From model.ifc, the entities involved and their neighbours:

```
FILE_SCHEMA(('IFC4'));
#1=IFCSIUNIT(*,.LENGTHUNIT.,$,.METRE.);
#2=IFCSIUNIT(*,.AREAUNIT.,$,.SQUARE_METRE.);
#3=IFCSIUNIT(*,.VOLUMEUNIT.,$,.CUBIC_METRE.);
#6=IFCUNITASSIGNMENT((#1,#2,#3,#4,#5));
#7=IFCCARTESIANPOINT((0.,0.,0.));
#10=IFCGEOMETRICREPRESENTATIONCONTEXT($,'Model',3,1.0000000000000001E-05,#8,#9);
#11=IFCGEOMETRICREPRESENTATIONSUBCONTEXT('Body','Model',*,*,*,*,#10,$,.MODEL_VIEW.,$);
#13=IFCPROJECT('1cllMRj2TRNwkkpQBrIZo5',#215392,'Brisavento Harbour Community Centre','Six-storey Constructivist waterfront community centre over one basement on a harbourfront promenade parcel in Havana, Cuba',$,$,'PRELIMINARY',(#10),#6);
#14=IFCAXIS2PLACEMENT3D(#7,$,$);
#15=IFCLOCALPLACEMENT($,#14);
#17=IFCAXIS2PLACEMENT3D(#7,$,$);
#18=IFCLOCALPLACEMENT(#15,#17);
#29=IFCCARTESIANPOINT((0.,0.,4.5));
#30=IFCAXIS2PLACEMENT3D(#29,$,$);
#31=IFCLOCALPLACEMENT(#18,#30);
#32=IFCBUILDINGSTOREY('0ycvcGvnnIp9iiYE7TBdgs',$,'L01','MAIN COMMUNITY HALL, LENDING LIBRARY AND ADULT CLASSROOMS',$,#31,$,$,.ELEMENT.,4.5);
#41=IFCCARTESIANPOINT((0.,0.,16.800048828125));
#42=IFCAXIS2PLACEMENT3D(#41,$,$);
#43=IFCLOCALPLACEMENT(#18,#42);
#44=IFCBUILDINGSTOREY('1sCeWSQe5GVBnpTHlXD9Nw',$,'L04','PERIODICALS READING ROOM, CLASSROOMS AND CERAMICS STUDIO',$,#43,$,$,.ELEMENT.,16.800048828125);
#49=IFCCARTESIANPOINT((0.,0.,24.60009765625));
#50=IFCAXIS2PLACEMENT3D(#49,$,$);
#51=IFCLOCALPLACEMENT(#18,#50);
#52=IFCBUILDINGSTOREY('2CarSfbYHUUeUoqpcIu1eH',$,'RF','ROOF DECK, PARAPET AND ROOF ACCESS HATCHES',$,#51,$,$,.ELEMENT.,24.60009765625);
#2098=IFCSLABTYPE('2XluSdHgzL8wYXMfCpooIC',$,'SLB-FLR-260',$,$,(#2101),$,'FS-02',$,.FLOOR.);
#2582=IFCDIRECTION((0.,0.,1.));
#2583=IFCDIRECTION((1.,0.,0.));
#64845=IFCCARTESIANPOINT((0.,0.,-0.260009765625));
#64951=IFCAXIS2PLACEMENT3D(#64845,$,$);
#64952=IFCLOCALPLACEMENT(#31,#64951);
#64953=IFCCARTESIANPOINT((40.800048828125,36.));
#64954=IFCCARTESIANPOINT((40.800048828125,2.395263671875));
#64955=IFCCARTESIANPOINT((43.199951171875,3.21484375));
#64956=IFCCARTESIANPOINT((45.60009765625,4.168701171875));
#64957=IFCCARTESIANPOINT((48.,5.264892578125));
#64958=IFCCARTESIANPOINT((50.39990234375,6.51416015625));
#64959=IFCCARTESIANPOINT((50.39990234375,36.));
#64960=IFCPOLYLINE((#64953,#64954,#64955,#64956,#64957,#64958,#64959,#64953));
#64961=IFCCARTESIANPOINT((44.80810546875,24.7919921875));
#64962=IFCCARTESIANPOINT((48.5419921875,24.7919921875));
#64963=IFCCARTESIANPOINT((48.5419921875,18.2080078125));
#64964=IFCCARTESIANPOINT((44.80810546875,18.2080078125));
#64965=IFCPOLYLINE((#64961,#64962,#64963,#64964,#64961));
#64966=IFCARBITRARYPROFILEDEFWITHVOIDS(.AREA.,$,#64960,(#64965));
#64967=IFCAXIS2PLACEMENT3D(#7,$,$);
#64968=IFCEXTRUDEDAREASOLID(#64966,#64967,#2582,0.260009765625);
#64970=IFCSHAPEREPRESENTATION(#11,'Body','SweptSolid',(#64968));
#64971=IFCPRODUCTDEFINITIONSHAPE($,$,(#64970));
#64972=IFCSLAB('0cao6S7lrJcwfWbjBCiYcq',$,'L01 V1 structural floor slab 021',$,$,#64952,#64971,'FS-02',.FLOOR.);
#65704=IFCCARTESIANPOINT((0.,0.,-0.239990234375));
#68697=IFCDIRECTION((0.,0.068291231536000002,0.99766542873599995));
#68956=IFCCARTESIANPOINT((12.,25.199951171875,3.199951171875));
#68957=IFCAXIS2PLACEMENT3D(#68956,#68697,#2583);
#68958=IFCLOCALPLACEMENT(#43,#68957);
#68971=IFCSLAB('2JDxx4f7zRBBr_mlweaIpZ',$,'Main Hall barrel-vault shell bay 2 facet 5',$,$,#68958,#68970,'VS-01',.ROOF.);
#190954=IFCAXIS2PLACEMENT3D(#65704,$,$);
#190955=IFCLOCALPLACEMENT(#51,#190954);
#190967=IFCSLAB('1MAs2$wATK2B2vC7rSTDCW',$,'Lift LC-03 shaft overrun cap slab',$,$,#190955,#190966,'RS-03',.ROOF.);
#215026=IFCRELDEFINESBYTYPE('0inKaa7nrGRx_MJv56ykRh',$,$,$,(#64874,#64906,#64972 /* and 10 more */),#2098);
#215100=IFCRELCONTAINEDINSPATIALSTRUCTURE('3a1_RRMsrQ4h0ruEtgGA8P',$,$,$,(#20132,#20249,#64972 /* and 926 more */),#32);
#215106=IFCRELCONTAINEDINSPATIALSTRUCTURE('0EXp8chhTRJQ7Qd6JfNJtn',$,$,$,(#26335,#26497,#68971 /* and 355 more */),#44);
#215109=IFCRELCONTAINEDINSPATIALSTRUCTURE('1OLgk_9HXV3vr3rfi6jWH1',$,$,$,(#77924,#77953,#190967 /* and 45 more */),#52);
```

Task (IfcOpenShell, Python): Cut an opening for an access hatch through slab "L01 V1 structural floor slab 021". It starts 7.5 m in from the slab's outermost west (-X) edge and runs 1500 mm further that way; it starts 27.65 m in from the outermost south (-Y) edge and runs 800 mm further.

```python
import numpy as np
import ifcopenshell
import ifcopenshell.api.feature
import ifcopenshell.api.geometry
import ifcopenshell.api.root
import ifcopenshell.geom
import ifcopenshell.util.placement
import ifcopenshell.util.representation
import ifcopenshell.util.shape
import ifcopenshell.util.unit

model = ifcopenshell.open("model.ifc")
unit_scale = ifcopenshell.util.unit.calculate_unit_scale(model)
settings = ifcopenshell.geom.settings()


def volume(element):
    """Net volume in cubic metres, openings subtracted."""
    shape = ifcopenshell.geom.create_shape(settings, element)
    return ifcopenshell.util.shape.get_volume(shape.geometry)


slab = model.by_id(64972)
before = volume(slab)

# Extent in the slab's own axes, in metres. The edges named are its -X and -Y sides.
slab_shape = ifcopenshell.geom.create_shape(settings, slab)
vertices = ifcopenshell.util.shape.get_vertices(slab_shape.geometry)
x_min, y_min, bottom = vertices.min(axis=0)
top = vertices[:, 2].max()

opening = ifcopenshell.api.root.create_entity(model, ifc_class="IfcOpeningElement", name="Access hatch opening", predefined_type="OPENING")
context = ifcopenshell.util.representation.get_context(model, "Model", "Body", "MODEL_VIEW")
width, depth = 1.5, 0.8
outline = [(0.0, 0.0), (width, 0.0), (width, depth), (0.0, depth), (0.0, 0.0)]
# Overshoot both faces by 50 mm so the cut is clean.
shape = ifcopenshell.api.geometry.add_slab_representation(
    model, context=context, depth=top - bottom + 0.1, polyline=outline
)
ifcopenshell.api.geometry.assign_representation(model, product=opening, representation=shape)

matrix = ifcopenshell.util.placement.get_local_placement(slab.ObjectPlacement)
matrix[:, 3] = matrix @ np.append(np.array([x_min + 7.5, y_min + 27.65, bottom - 0.05]) / unit_scale, 1.0)
ifcopenshell.api.geometry.edit_object_placement(model, product=opening, matrix=matrix, is_si=False)
ifcopenshell.api.feature.add_feature(model, feature=opening, element=slab)

after = volume(slab)

print(f"slab volume {before:.3f} -> {after:.3f} m3")

model.write("model_edited.ifc")
```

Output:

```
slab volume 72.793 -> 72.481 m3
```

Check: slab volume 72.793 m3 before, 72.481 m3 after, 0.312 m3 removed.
